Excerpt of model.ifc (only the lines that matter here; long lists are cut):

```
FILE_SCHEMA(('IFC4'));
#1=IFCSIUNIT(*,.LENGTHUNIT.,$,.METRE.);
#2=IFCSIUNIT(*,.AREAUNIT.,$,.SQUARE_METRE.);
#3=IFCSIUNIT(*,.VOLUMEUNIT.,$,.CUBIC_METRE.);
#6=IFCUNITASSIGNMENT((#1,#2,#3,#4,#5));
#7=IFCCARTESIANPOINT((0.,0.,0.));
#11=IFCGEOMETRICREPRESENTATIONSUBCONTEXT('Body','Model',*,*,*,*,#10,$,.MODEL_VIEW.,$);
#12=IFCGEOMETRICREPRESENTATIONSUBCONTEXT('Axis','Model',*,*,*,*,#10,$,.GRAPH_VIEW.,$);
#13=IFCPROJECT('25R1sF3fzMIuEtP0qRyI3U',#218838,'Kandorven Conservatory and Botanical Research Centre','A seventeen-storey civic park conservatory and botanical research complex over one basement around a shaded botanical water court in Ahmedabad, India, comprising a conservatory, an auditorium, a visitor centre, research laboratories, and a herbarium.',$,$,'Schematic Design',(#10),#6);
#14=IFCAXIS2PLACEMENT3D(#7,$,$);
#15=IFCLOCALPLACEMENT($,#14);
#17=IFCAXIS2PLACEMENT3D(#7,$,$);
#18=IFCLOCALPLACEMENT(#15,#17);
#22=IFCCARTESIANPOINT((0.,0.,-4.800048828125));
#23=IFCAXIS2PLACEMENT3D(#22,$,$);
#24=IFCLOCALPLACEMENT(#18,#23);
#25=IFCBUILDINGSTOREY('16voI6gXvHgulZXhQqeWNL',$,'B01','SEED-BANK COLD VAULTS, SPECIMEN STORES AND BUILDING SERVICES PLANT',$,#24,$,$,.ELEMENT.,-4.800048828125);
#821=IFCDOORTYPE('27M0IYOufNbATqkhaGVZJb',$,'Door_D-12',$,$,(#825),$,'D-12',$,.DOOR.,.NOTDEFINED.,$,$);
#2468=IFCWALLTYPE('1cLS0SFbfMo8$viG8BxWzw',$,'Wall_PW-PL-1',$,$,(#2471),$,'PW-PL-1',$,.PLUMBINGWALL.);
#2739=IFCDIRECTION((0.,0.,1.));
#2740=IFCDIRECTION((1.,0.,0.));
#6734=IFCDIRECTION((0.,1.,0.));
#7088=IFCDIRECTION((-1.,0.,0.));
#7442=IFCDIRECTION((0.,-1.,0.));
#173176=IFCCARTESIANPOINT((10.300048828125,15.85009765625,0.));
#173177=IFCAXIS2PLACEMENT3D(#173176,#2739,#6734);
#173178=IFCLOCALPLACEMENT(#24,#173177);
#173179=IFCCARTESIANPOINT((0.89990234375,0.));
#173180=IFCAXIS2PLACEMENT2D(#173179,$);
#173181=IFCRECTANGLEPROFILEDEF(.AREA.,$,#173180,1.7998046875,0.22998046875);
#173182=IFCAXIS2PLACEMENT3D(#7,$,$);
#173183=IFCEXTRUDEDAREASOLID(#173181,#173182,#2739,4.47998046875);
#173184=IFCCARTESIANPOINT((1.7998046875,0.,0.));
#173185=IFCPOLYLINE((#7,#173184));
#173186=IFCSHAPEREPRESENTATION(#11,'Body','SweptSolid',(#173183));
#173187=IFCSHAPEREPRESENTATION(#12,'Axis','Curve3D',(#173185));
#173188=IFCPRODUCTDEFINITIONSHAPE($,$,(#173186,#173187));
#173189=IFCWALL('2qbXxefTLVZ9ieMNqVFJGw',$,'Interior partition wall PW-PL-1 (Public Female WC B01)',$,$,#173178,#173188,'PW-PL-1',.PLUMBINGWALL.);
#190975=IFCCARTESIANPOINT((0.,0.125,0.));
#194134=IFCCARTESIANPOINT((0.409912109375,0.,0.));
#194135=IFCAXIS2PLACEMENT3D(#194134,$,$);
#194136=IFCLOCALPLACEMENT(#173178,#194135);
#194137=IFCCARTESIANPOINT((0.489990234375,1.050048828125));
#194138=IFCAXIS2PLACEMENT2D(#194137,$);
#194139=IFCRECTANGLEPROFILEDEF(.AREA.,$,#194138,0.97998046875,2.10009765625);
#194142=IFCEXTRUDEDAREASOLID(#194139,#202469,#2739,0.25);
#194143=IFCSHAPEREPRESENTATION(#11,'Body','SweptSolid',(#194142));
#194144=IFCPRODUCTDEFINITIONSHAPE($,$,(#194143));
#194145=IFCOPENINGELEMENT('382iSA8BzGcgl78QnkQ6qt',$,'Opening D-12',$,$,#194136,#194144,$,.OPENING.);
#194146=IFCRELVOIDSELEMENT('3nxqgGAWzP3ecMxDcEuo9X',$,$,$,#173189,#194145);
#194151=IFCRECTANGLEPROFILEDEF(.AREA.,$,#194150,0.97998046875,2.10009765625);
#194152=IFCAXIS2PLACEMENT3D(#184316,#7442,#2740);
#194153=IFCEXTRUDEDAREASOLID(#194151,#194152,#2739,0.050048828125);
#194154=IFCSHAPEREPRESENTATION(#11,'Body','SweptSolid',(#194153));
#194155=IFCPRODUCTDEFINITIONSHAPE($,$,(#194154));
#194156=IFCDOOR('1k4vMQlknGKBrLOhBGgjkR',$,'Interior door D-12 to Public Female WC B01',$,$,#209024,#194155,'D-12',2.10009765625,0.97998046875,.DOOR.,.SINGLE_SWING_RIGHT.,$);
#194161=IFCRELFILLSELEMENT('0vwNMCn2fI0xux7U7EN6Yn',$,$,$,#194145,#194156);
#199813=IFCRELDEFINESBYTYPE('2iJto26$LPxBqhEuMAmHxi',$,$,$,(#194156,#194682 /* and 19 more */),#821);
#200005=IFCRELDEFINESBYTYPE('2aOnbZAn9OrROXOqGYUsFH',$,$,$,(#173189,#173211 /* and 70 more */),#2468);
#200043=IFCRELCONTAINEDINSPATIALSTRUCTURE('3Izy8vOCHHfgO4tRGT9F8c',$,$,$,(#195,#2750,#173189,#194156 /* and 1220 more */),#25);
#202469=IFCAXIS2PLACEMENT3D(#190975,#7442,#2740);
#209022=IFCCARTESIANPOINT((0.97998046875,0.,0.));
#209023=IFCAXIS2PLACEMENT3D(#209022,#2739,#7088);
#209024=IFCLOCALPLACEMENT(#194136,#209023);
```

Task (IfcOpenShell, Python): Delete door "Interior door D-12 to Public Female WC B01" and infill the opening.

```python
import ifcopenshell
import ifcopenshell.api.feature
import ifcopenshell.api.root
import ifcopenshell.geom
import ifcopenshell.util.shape

model = ifcopenshell.open("model.ifc")
settings = ifcopenshell.geom.settings()


def volume(element):
    """Net volume in cubic metres, openings subtracted."""
    shape = ifcopenshell.geom.create_shape(settings, element)
    return ifcopenshell.util.shape.get_volume(shape.geometry)


door = model.by_id(194156)
opening = door.FillsVoids[0].RelatingOpeningElement
wall = opening.VoidsElements[0].RelatingBuildingElement
before = volume(wall)

ifcopenshell.api.root.remove_product(model, product=door)
ifcopenshell.api.feature.remove_feature(model, feature=opening)

after = volume(wall)

print(f"wall volume {before:.3f} -> {after:.3f} m3")

model.write("model-out.ifc")
```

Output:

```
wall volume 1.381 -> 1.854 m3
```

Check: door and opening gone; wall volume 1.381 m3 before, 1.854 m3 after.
